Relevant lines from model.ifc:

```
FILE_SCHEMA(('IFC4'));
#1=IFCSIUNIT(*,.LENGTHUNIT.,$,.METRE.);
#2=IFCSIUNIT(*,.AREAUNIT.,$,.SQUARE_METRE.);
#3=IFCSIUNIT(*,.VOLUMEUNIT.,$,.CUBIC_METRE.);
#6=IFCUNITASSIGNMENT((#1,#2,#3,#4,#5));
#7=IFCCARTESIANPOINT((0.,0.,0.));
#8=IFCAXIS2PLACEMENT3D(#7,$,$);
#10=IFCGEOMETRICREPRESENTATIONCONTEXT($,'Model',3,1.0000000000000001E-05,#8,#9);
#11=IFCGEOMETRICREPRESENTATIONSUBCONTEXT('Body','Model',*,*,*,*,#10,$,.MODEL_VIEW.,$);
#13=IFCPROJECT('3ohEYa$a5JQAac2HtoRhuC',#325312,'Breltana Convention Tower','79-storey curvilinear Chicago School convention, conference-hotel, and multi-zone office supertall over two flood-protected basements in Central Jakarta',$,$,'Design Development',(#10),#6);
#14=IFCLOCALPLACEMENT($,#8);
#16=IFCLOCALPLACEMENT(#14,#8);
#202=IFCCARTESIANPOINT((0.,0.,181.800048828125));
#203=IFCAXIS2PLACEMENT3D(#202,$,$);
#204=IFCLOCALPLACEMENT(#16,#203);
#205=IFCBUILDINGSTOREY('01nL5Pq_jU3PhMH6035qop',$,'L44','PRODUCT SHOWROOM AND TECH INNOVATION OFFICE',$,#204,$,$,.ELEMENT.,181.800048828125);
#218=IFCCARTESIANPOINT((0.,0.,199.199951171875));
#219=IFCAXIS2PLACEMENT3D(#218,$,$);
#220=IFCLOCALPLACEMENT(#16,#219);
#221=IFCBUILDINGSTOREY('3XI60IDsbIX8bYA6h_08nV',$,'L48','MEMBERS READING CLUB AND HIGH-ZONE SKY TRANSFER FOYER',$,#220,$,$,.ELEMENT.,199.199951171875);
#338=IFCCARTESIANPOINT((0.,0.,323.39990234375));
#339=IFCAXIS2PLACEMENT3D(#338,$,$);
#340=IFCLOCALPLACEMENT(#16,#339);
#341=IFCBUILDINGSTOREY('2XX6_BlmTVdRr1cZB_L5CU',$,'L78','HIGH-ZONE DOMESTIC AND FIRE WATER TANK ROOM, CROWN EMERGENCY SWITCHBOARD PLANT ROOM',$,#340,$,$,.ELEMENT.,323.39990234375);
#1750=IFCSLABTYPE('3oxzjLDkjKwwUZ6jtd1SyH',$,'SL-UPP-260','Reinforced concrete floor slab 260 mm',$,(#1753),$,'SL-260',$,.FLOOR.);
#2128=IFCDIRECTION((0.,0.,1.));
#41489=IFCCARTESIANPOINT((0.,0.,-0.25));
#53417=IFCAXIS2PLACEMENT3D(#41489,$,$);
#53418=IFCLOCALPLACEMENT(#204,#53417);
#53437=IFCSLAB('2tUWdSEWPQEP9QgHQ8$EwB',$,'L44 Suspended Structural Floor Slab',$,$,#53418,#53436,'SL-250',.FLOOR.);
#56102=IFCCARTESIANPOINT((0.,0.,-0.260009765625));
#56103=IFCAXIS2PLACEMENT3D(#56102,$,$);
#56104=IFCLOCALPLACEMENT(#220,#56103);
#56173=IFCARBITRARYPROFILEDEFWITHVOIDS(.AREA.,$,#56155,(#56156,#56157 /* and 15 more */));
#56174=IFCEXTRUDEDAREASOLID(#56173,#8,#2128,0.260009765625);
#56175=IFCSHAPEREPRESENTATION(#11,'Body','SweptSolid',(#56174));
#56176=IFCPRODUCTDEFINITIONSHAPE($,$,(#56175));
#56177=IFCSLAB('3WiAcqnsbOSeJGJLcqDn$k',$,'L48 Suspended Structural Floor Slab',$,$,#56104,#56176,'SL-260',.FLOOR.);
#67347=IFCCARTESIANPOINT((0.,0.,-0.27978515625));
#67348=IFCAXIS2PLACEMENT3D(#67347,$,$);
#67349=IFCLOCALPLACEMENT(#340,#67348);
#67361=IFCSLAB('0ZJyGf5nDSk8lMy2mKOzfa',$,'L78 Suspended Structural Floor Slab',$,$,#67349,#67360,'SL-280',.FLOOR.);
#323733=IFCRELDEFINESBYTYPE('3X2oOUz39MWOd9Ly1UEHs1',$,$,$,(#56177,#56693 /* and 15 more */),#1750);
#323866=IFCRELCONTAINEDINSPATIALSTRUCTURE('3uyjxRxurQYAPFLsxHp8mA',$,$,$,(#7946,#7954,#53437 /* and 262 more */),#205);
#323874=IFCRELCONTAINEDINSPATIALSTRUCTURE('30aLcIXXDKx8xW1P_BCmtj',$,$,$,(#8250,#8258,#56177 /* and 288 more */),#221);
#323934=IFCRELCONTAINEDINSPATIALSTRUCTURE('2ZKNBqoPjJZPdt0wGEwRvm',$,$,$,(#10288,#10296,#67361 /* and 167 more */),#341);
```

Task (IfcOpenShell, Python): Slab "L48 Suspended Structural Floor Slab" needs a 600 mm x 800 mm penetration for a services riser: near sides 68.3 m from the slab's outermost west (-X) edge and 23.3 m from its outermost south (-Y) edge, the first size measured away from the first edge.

```python
import numpy as np
import ifcopenshell
import ifcopenshell.api.feature
import ifcopenshell.api.geometry
import ifcopenshell.api.root
import ifcopenshell.geom
import ifcopenshell.util.placement
import ifcopenshell.util.representation
import ifcopenshell.util.shape
import ifcopenshell.util.unit

model = ifcopenshell.open("model.ifc")
unit_scale = ifcopenshell.util.unit.calculate_unit_scale(model)
settings = ifcopenshell.geom.settings()


def volume(element):
    """Net volume in cubic metres, openings subtracted."""
    shape = ifcopenshell.geom.create_shape(settings, element)
    return ifcopenshell.util.shape.get_volume(shape.geometry)


slab = model.by_id(56177)
before = volume(slab)

# Extent in the slab's own axes, in metres. The edges named are its -X and -Y sides.
slab_shape = ifcopenshell.geom.create_shape(settings, slab)
vertices = ifcopenshell.util.shape.get_vertices(slab_shape.geometry)
x_min, y_min, bottom = vertices.min(axis=0)
top = vertices[:, 2].max()

opening = ifcopenshell.api.root.create_entity(model, ifc_class="IfcOpeningElement", name="Services riser opening", predefined_type="OPENING")
context = ifcopenshell.util.representation.get_context(model, "Model", "Body", "MODEL_VIEW")
width, depth = 0.6, 0.8
outline = [(0.0, 0.0), (width, 0.0), (width, depth), (0.0, depth), (0.0, 0.0)]
# Overshoot both faces by 50 mm so the cut is clean.
shape = ifcopenshell.api.geometry.add_slab_representation(
    model, context=context, depth=top - bottom + 0.1, polyline=outline
)
ifcopenshell.api.geometry.assign_representation(model, product=opening, representation=shape)

matrix = ifcopenshell.util.placement.get_local_placement(slab.ObjectPlacement)
matrix[:, 3] = matrix @ np.append(np.array([x_min + 68.3, y_min + 23.3, bottom - 0.05]) / unit_scale, 1.0)
ifcopenshell.api.geometry.edit_object_placement(model, product=opening, matrix=matrix, is_si=False)
ifcopenshell.api.feature.add_feature(model, feature=opening, element=slab)

after = volume(slab)

print(f"slab volume {before:.3f} -> {after:.3f} m3")

model.write("model_v2.ifc")
```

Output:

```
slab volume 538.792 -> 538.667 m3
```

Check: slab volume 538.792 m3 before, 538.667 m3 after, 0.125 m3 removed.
